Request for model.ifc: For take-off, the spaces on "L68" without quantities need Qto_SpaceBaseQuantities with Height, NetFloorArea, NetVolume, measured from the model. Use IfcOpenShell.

First a look at what the model holds.

```python
import ifcopenshell
import ifcopenshell.util.element
import ifcopenshell.util.unit

model = ifcopenshell.open("model.ifc")
print(model.schema)
for unit_type in ("LENGTHUNIT", "AREAUNIT", "VOLUMEUNIT"):
    print(unit_type, ifcopenshell.util.unit.calculate_unit_scale(model, unit_type))
storey = next(s for s in model.by_type("IfcBuildingStorey") if s.Name == "L68")
spaces = [e for e in ifcopenshell.util.element.get_decomposition(storey) if e.is_a("IfcSpace")]
for e in sorted(spaces, key=lambda e: e.id()):
    print(e.id(), e.is_a(), e.Name, list(ifcopenshell.util.element.get_psets(e, qtos_only=True)), sep=" | ")
```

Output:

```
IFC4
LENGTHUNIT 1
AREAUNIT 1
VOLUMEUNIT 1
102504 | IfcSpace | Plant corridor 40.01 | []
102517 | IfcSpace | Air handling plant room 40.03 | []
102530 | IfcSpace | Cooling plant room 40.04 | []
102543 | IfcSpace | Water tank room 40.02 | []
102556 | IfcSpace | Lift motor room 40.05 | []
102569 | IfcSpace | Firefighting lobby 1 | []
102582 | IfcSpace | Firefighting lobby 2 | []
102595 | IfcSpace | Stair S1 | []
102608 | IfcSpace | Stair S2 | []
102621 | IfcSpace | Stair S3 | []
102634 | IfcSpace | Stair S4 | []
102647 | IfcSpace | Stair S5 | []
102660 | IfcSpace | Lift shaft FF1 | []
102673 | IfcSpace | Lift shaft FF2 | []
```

```python
import ifcopenshell
import ifcopenshell.api.pset
import ifcopenshell.geom
import ifcopenshell.util.element
import ifcopenshell.util.shape
import ifcopenshell.util.unit

model = ifcopenshell.open("model.ifc")
unit_scale = ifcopenshell.util.unit.calculate_unit_scale(model)
area_scale = ifcopenshell.util.unit.calculate_unit_scale(model, "AREAUNIT")
volume_scale = ifcopenshell.util.unit.calculate_unit_scale(model, "VOLUMEUNIT")
settings = ifcopenshell.geom.settings()

storey = next(s for s in model.by_type("IfcBuildingStorey") if s.Name == "L68")
spaces = [e for e in ifcopenshell.util.element.get_decomposition(storey) if e.is_a("IfcSpace")]

for e in sorted(spaces, key=lambda e: e.id()):
    if ifcopenshell.util.element.get_psets(e, qtos_only=True, should_inherit=False):
        continue
    # Geometry comes back in metres, in the element's own axes.
    shape = ifcopenshell.geom.create_shape(settings, e)
    values = {
        "Height": ifcopenshell.util.shape.get_z(shape.geometry) / unit_scale,
        "NetFloorArea": ifcopenshell.util.shape.get_footprint_area(shape.geometry) / area_scale,
        "NetVolume": ifcopenshell.util.shape.get_volume(shape.geometry) / volume_scale,
    }
    qto = ifcopenshell.api.pset.add_qto(model, product=e, name="Qto_SpaceBaseQuantities")
    ifcopenshell.api.pset.edit_qto(model, qto=qto, properties=values)
    print(e.id(), {k: round(v, 3) for k, v in values.items()})

model.write("model_v2.ifc")
```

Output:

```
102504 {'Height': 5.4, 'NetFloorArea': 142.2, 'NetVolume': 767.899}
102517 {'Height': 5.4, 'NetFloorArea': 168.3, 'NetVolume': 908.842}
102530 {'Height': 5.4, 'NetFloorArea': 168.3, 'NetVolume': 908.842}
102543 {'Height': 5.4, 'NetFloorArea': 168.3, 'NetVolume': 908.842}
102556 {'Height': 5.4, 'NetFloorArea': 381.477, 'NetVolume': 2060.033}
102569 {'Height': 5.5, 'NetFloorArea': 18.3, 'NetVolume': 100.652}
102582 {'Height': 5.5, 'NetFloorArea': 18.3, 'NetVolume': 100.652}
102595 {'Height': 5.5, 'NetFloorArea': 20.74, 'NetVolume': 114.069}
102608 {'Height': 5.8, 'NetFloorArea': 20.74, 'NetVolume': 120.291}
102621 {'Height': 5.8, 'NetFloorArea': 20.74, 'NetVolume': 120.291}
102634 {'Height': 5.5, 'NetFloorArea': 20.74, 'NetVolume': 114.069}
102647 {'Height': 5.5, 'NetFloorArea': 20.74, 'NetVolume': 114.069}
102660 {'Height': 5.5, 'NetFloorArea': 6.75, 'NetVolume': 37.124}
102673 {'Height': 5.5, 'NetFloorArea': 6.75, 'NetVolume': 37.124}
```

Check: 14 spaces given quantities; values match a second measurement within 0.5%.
